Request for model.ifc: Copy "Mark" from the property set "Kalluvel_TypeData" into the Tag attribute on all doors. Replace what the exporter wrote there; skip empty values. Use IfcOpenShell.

First a look at what the model holds.

```python
import ifcopenshell
import ifcopenshell.util.element

model = ifcopenshell.open("model.ifc")
print(model.schema)
doors = model.by_type("IfcDoor")
print(len(doors), "doors")
for e in doors[:8]:
    source = ifcopenshell.util.element.get_pset(e, "Kalluvel_TypeData", "Mark")
    target = e.Tag
    print(e.id(), repr(source), repr(target), sep=" | ")
```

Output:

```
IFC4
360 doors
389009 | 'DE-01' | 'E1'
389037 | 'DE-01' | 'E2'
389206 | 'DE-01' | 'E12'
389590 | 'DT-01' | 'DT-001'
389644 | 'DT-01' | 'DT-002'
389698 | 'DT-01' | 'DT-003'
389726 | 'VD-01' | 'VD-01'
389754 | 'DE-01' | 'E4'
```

```python
import ifcopenshell
import ifcopenshell.util.element

model = ifcopenshell.open("model.ifc")

count = 0
for e in model.by_type("IfcDoor"):
    value = ifcopenshell.util.element.get_pset(e, "Kalluvel_TypeData", "Mark")
    current = e.Tag
    if not value or not value.strip() or current == value:
        continue
    e.Tag = value
    count += 1

print(count, "doors updated")

model.write("model_v2.ifc")
```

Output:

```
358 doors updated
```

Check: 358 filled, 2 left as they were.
